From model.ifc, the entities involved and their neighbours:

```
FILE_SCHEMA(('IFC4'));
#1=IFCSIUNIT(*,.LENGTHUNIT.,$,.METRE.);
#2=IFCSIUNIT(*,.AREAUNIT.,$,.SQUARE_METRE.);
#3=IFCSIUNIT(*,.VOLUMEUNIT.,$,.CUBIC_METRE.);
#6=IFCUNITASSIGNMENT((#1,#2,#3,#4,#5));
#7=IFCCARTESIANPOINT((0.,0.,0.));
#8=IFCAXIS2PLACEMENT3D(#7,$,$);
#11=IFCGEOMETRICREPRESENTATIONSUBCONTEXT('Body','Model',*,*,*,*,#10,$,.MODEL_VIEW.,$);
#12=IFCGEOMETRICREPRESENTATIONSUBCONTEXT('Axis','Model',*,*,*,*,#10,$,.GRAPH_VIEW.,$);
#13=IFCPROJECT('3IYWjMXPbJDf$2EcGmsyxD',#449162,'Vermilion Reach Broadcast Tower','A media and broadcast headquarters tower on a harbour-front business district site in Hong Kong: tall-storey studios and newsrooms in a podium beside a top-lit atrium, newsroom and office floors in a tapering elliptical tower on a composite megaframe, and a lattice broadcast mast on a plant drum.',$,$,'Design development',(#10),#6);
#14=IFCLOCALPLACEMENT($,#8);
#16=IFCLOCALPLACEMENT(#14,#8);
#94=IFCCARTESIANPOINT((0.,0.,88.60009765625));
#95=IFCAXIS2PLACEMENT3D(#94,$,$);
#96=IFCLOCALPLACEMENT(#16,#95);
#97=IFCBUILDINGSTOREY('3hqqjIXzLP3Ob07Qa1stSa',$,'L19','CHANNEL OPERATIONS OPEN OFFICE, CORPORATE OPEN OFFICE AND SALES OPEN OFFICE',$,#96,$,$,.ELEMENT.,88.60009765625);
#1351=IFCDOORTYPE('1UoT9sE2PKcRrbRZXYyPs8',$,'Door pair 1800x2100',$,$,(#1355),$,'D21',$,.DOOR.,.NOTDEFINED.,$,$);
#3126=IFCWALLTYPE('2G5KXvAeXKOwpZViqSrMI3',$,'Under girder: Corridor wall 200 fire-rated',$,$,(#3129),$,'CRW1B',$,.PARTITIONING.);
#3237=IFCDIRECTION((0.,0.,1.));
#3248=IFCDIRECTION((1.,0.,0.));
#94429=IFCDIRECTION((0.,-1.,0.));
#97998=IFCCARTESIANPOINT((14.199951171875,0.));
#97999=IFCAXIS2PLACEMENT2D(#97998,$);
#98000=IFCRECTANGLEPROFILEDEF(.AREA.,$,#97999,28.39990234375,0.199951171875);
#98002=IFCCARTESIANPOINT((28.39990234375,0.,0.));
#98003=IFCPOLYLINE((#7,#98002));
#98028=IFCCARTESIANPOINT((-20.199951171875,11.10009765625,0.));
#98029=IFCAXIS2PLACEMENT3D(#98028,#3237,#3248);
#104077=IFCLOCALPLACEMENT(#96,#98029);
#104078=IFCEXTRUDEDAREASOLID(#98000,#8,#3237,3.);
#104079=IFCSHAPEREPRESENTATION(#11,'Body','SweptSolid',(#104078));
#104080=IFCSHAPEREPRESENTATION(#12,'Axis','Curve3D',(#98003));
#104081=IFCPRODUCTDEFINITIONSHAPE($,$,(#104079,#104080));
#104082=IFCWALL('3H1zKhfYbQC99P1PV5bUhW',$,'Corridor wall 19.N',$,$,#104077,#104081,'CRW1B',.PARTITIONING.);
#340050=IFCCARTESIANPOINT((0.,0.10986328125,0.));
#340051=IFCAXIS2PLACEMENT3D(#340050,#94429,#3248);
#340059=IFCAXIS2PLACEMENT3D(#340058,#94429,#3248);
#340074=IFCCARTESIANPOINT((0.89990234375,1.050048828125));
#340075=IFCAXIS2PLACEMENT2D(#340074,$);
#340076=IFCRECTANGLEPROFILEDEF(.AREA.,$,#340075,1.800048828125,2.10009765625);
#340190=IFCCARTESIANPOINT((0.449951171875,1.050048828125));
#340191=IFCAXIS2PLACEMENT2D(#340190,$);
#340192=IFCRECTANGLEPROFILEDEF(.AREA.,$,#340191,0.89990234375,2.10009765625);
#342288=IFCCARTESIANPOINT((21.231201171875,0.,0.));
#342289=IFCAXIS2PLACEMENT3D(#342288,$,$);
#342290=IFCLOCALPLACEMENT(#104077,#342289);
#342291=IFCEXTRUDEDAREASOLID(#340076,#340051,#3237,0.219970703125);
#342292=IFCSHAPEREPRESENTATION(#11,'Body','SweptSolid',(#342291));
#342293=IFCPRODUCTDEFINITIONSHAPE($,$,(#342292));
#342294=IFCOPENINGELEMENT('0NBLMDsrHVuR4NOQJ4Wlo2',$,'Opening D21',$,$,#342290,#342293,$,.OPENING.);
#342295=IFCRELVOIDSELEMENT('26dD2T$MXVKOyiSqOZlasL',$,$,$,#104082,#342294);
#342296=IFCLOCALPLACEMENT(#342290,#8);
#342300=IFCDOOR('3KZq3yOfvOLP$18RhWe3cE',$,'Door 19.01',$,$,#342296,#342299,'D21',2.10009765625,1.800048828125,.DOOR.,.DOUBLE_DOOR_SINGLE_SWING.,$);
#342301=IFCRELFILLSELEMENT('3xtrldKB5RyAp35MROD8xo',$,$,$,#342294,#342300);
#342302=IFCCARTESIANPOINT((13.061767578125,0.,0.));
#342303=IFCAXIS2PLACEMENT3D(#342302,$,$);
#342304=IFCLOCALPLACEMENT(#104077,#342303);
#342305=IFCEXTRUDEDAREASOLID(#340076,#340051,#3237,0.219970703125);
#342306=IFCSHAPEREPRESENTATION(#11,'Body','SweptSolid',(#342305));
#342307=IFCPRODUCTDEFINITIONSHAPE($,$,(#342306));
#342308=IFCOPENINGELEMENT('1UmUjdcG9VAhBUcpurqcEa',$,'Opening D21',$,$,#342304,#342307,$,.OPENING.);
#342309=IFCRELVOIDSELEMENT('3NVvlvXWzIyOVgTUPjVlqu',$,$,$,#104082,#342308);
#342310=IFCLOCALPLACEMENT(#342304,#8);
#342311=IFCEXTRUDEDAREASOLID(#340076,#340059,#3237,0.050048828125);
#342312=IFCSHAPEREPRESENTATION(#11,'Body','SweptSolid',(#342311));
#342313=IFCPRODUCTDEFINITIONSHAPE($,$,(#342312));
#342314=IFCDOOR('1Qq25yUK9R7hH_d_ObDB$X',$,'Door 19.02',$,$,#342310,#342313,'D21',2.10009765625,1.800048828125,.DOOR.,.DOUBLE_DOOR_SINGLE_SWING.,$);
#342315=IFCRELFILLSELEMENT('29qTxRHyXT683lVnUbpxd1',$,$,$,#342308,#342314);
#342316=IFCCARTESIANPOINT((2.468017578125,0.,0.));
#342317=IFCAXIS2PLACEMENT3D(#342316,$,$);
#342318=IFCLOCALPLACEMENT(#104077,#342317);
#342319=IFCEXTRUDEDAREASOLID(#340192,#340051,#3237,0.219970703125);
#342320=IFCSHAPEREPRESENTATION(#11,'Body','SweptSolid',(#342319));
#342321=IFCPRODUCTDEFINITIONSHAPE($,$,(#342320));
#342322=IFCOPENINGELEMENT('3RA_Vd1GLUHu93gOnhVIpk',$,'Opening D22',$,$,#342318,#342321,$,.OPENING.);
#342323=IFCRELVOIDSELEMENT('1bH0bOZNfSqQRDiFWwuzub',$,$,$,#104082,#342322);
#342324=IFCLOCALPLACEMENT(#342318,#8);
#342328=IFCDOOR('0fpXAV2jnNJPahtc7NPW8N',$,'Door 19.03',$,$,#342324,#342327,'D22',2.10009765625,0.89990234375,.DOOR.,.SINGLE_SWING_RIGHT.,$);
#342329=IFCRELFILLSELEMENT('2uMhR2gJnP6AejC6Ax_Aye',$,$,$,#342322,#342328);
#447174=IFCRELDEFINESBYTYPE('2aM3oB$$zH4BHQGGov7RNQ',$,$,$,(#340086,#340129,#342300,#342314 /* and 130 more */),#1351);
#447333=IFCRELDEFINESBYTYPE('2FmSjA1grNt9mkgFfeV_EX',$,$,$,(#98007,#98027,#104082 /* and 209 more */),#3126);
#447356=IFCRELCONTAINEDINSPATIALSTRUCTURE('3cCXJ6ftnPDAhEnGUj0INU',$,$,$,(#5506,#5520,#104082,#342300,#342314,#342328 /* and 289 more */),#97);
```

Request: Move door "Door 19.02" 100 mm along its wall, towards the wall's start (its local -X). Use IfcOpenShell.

```python
import ifcopenshell
import ifcopenshell.api.geometry
import ifcopenshell.util.placement

model = ifcopenshell.open("model.ifc")

door = model.by_guid("1Qq25yUK9R7hH_d_ObDB$X")
opening = door.FillsVoids[0].RelatingOpeningElement
wall = opening.VoidsElements[0].RelatingBuildingElement

wall_matrix = ifcopenshell.util.placement.get_local_placement(wall.ObjectPlacement)
shift = wall_matrix[:3, 0] * -0.1
before = ifcopenshell.util.placement.get_local_placement(door.ObjectPlacement)[:3, 3].copy()

# The door is placed relative to its opening, so it follows when the opening moves.
matrix = ifcopenshell.util.placement.get_local_placement(opening.ObjectPlacement)
matrix[:3, 3] += shift
ifcopenshell.api.geometry.edit_object_placement(
    model, product=opening, matrix=matrix, is_si=False, should_transform_children=True
)

after = ifcopenshell.util.placement.get_local_placement(door.ObjectPlacement)[:3, 3]
print("door moved by", (after - before).round(3) + 0.0)

model.write("model-out.ifc")
```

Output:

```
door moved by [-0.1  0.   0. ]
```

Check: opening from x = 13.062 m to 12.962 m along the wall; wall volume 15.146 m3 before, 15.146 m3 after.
